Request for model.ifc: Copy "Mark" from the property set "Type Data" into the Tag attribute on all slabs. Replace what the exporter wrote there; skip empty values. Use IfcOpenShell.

First a look at what the model holds.

```python
import ifcopenshell
import ifcopenshell.util.element

model = ifcopenshell.open("model.ifc")
print(model.schema)
slabs = model.by_type("IfcSlab")
print(len(slabs), "slabs")
for e in slabs[:8]:
    source = ifcopenshell.util.element.get_pset(e, "Type Data", "Mark")
    target = e.Tag
    print(e.id(), repr(source), repr(target), sep=" | ")
```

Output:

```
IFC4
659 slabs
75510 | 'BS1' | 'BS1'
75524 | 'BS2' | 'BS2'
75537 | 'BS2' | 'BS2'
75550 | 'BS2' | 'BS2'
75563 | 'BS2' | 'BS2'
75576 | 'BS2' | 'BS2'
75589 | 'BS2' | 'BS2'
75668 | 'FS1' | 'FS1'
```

```python
import ifcopenshell
import ifcopenshell.util.element

model = ifcopenshell.open("model.ifc")

count = 0
for e in model.by_type("IfcSlab"):
    value = ifcopenshell.util.element.get_pset(e, "Type Data", "Mark")
    current = e.Tag
    if not value or not value.strip() or current == value:
        continue
    e.Tag = value
    count += 1

print(count, "slabs updated")

model.write("model-out.ifc")
```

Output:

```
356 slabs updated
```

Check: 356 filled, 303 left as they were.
